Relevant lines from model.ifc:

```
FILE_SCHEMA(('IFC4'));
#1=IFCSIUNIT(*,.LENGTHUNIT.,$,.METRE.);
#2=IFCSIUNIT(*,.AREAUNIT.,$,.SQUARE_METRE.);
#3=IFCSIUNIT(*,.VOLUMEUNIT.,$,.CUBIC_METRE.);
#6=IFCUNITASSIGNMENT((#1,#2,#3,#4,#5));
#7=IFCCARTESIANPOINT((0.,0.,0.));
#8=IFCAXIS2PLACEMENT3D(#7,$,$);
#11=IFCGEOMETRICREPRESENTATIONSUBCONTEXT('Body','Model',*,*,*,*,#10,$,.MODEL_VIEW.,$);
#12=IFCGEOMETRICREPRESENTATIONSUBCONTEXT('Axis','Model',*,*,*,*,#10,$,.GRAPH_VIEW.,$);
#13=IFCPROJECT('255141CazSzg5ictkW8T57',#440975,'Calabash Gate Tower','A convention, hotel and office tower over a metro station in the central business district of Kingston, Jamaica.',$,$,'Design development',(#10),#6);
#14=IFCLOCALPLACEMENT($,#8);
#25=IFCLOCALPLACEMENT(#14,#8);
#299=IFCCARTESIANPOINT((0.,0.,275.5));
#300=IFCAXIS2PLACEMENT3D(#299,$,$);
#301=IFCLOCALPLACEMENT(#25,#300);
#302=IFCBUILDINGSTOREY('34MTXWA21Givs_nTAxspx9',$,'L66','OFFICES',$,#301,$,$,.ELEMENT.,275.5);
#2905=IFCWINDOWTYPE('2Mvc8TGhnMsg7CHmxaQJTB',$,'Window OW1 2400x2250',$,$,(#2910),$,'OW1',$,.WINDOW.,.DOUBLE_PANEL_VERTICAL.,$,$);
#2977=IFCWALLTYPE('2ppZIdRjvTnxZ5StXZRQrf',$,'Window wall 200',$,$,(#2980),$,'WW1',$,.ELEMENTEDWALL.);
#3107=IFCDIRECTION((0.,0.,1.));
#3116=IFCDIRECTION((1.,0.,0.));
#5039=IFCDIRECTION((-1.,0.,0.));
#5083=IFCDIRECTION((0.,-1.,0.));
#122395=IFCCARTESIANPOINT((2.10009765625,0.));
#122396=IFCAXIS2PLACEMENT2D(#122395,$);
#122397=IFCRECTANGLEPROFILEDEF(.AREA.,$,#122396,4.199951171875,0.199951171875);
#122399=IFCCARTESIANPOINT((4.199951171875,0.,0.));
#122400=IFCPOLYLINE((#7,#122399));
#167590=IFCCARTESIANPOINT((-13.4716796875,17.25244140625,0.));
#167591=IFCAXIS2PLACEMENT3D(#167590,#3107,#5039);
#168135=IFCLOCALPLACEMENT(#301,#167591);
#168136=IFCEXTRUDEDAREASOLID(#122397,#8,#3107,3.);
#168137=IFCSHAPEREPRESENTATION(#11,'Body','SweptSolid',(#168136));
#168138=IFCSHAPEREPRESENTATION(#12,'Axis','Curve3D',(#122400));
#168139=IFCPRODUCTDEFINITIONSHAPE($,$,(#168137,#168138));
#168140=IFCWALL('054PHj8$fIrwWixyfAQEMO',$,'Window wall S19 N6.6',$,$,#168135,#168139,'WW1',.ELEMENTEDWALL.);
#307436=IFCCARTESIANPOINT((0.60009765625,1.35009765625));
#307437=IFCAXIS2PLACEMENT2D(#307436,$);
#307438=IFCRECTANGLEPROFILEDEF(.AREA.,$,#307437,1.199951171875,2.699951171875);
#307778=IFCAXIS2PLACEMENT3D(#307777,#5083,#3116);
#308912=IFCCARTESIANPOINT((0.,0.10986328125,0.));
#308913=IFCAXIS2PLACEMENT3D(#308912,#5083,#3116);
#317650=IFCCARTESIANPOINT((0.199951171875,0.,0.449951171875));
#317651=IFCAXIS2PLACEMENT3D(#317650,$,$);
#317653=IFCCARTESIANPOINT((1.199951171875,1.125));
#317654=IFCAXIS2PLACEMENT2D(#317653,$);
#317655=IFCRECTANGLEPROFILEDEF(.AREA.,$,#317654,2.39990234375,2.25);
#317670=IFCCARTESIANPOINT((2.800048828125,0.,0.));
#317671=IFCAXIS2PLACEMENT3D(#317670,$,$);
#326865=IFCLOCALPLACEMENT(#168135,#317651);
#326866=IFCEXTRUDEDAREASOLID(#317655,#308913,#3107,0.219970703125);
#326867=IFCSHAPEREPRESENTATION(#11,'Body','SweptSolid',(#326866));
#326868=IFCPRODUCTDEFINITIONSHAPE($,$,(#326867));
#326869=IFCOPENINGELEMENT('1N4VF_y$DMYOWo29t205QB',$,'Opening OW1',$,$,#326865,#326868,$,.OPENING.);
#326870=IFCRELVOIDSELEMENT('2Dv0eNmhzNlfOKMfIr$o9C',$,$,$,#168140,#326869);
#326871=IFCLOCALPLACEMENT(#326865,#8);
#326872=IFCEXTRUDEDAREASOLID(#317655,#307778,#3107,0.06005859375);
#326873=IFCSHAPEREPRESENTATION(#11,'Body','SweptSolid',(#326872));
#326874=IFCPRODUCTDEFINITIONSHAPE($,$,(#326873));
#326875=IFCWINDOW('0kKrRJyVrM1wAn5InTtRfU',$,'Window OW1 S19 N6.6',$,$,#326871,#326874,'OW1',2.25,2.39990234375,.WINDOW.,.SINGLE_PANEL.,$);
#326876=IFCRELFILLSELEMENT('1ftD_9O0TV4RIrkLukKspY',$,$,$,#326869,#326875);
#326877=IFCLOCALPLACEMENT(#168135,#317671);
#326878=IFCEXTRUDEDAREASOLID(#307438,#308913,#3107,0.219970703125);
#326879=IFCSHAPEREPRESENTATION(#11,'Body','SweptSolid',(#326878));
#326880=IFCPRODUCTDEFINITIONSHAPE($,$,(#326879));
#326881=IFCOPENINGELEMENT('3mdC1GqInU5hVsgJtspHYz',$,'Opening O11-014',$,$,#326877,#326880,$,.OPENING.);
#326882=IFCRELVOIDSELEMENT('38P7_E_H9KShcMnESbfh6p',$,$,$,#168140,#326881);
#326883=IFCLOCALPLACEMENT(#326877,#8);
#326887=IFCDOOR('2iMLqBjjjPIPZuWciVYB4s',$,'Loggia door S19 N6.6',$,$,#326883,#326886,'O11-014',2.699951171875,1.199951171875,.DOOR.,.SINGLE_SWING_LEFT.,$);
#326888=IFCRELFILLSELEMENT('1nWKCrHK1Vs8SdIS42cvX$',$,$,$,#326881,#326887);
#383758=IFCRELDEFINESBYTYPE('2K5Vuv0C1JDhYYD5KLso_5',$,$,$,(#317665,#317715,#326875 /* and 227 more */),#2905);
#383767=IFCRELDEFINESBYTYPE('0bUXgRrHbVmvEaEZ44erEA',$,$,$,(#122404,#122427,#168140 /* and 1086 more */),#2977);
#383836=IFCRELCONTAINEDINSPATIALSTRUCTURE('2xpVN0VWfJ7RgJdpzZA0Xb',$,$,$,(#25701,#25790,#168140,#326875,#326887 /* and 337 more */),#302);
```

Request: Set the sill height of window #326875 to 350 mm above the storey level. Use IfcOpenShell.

```python
import numpy as np
import ifcopenshell
import ifcopenshell.api.geometry
import ifcopenshell.geom
import ifcopenshell.util.element
import ifcopenshell.util.placement
import ifcopenshell.util.shape
import ifcopenshell.util.unit

model = ifcopenshell.open("model.ifc")
unit_scale = ifcopenshell.util.unit.calculate_unit_scale(model)

window = model.by_guid("0kKrRJyVrM1wAn5InTtRfU")
opening = window.FillsVoids[0].RelatingOpeningElement
storey = ifcopenshell.util.element.get_container(window, ifc_class="IfcBuildingStorey")
level = ifcopenshell.util.placement.get_local_placement(storey.ObjectPlacement)[2, 3]

# The opening's origin need not be at the sill, so measure its lowest point.
shape = ifcopenshell.geom.create_shape(ifcopenshell.geom.settings(), opening)
bottom = ifcopenshell.util.shape.get_shape_bottom_elevation(shape, shape.geometry) / unit_scale
dz = level + 0.35 / unit_scale - bottom

shift = np.array([0.0, 0.0, dz])
# The window is placed relative to its opening, so it follows when the opening moves.
matrix = ifcopenshell.util.placement.get_local_placement(opening.ObjectPlacement)
matrix[:3, 3] += shift
ifcopenshell.api.geometry.edit_object_placement(
    model, product=opening, matrix=matrix, is_si=False, should_transform_children=True
)

print(f"moved by {dz * unit_scale:+.3f} m")

model.write("model_edited.ifc")
```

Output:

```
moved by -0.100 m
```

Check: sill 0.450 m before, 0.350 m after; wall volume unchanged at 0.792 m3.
